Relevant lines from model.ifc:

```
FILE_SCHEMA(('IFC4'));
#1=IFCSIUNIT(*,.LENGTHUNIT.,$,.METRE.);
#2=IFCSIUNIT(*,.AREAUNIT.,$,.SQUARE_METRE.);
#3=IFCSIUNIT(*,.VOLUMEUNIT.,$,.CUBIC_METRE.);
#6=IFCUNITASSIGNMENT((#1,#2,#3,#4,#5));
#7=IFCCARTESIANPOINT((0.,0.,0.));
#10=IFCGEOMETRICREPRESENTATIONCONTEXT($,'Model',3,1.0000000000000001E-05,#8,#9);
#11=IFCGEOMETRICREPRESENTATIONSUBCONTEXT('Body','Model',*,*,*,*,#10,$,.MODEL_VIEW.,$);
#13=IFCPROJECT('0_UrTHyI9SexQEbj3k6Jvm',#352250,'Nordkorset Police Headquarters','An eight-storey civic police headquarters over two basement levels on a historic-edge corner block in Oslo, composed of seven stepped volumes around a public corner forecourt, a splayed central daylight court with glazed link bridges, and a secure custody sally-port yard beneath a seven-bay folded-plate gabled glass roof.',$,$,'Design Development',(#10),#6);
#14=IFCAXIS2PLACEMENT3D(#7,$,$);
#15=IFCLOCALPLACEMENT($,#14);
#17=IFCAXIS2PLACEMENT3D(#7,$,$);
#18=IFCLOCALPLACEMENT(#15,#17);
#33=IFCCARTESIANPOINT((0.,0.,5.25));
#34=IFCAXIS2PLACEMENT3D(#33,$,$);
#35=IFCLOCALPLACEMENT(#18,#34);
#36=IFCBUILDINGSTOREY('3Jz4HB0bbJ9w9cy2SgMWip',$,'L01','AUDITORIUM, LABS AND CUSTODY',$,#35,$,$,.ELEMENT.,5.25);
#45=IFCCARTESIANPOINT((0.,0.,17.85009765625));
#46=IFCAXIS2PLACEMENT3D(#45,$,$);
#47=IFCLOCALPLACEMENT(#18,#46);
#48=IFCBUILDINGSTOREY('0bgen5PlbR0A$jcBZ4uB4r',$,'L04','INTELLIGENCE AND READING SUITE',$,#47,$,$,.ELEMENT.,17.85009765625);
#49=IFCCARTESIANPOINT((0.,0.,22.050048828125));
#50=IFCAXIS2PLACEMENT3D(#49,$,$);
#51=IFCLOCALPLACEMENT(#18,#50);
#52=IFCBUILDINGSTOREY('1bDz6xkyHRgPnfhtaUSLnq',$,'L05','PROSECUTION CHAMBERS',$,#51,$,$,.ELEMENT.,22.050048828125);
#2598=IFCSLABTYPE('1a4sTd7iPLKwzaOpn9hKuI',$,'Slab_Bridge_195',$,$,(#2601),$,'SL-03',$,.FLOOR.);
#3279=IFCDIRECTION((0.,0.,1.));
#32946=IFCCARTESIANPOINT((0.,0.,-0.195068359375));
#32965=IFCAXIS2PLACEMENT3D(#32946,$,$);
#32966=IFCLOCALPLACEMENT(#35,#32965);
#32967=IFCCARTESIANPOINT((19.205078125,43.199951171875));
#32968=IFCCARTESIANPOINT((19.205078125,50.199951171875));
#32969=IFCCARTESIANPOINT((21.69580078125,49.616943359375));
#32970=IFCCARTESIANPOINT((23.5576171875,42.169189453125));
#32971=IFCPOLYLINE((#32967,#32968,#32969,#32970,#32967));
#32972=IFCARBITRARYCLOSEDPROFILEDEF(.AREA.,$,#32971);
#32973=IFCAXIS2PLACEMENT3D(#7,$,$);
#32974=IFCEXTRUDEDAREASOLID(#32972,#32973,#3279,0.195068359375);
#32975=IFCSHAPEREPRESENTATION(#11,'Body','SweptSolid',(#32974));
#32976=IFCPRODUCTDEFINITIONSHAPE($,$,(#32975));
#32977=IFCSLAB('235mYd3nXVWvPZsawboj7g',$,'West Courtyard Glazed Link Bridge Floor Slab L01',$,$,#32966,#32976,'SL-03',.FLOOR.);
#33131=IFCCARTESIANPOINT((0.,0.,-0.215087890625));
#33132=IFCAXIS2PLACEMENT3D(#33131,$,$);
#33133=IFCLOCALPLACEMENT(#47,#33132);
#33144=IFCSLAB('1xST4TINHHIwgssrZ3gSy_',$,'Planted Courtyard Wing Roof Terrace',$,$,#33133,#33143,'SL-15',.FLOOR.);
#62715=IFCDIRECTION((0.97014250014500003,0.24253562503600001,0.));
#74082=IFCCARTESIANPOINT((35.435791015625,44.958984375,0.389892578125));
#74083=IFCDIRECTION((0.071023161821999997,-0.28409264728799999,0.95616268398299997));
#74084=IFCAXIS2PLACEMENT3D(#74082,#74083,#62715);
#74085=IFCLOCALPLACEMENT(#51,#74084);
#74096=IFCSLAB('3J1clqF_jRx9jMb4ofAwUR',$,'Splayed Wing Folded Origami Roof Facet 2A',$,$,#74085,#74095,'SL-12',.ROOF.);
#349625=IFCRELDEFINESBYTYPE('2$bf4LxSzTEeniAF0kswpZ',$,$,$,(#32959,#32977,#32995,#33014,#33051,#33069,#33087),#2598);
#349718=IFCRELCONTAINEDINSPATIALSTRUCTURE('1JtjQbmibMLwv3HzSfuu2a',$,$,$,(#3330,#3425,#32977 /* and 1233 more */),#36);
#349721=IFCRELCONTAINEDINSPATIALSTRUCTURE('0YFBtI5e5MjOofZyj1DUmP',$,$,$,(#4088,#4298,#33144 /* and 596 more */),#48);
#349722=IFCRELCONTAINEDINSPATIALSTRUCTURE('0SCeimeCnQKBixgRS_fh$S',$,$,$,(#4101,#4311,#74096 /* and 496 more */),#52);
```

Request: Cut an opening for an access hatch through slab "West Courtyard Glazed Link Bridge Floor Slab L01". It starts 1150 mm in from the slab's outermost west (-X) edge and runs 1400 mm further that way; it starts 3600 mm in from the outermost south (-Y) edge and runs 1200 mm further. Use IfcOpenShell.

```python
import numpy as np
import ifcopenshell
import ifcopenshell.api.feature
import ifcopenshell.api.geometry
import ifcopenshell.api.root
import ifcopenshell.geom
import ifcopenshell.util.placement
import ifcopenshell.util.representation
import ifcopenshell.util.shape
import ifcopenshell.util.unit

model = ifcopenshell.open("model.ifc")
unit_scale = ifcopenshell.util.unit.calculate_unit_scale(model)
settings = ifcopenshell.geom.settings()


def volume(element):
    """Net volume in cubic metres, openings subtracted."""
    shape = ifcopenshell.geom.create_shape(settings, element)
    return ifcopenshell.util.shape.get_volume(shape.geometry)


slab = model.by_guid("235mYd3nXVWvPZsawboj7g")
before = volume(slab)

# Extent in the slab's own axes, in metres. The edges named are its -X and -Y sides.
slab_shape = ifcopenshell.geom.create_shape(settings, slab)
vertices = ifcopenshell.util.shape.get_vertices(slab_shape.geometry)
x_min, y_min, bottom = vertices.min(axis=0)
top = vertices[:, 2].max()

opening = ifcopenshell.api.root.create_entity(model, ifc_class="IfcOpeningElement", name="Access hatch opening", predefined_type="OPENING")
context = ifcopenshell.util.representation.get_context(model, "Model", "Body", "MODEL_VIEW")
width, depth = 1.4, 1.2
outline = [(0.0, 0.0), (width, 0.0), (width, depth), (0.0, depth), (0.0, 0.0)]
# Overshoot both faces by 50 mm so the cut is clean.
shape = ifcopenshell.api.geometry.add_slab_representation(
    model, context=context, depth=top - bottom + 0.1, polyline=outline
)
ifcopenshell.api.geometry.assign_representation(model, product=opening, representation=shape)

matrix = ifcopenshell.util.placement.get_local_placement(slab.ObjectPlacement)
matrix[:, 3] = matrix @ np.append(np.array([x_min + 1.15, y_min + 3.6, bottom - 0.05]) / unit_scale, 1.0)
ifcopenshell.api.geometry.edit_object_placement(model, product=opening, matrix=matrix, is_si=False)
ifcopenshell.api.feature.add_feature(model, feature=opening, element=slab)

after = volume(slab)

print(f"slab volume {before:.3f} -> {after:.3f} m3")

model.write("model_v2.ifc")
```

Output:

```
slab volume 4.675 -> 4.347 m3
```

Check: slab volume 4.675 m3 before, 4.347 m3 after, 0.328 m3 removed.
